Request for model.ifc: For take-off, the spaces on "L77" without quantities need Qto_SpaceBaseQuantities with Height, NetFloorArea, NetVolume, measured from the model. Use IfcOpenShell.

First a look at what the model holds.

```python
import ifcopenshell
import ifcopenshell.util.element
import ifcopenshell.util.unit

model = ifcopenshell.open("model.ifc")
print(model.schema)
for unit_type in ("LENGTHUNIT", "AREAUNIT", "VOLUMEUNIT"):
    print(unit_type, ifcopenshell.util.unit.calculate_unit_scale(model, unit_type))
storey = next(s for s in model.by_type("IfcBuildingStorey") if s.Name == "L77")
spaces = [e for e in ifcopenshell.util.element.get_decomposition(storey) if e.is_a("IfcSpace")]
for e in sorted(spaces, key=lambda e: e.id()):
    print(e.id(), e.is_a(), e.Name, list(ifcopenshell.util.element.get_psets(e, qtos_only=True)), sep=" | ")
```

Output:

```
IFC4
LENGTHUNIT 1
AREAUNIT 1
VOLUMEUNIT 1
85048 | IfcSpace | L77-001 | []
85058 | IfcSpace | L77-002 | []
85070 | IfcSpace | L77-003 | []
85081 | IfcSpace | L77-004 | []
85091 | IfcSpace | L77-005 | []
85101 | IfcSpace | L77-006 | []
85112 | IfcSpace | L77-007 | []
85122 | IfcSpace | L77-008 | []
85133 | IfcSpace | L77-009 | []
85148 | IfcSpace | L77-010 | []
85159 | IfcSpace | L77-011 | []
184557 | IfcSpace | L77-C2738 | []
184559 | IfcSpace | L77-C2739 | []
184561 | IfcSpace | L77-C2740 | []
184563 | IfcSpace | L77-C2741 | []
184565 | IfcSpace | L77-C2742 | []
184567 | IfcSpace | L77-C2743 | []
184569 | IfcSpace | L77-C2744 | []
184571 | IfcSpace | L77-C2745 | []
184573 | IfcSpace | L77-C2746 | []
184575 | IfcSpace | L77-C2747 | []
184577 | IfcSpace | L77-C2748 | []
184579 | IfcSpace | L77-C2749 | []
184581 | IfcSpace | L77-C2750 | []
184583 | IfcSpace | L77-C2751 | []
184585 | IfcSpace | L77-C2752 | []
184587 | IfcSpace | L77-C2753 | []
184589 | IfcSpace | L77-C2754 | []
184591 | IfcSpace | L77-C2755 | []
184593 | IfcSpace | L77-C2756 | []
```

```python
import ifcopenshell
import ifcopenshell.api.pset
import ifcopenshell.geom
import ifcopenshell.util.element
import ifcopenshell.util.shape
import ifcopenshell.util.unit

model = ifcopenshell.open("model.ifc")
unit_scale = ifcopenshell.util.unit.calculate_unit_scale(model)
area_scale = ifcopenshell.util.unit.calculate_unit_scale(model, "AREAUNIT")
volume_scale = ifcopenshell.util.unit.calculate_unit_scale(model, "VOLUMEUNIT")
settings = ifcopenshell.geom.settings()

storey = next(s for s in model.by_type("IfcBuildingStorey") if s.Name == "L77")
spaces = [e for e in ifcopenshell.util.element.get_decomposition(storey) if e.is_a("IfcSpace")]

for e in sorted(spaces, key=lambda e: e.id()):
    if ifcopenshell.util.element.get_psets(e, qtos_only=True, should_inherit=False):
        continue
    # Geometry comes back in metres, in the element's own axes.
    shape = ifcopenshell.geom.create_shape(settings, e)
    values = {
        "Height": ifcopenshell.util.shape.get_z(shape.geometry) / unit_scale,
        "NetFloorArea": ifcopenshell.util.shape.get_footprint_area(shape.geometry) / area_scale,
        "NetVolume": ifcopenshell.util.shape.get_volume(shape.geometry) / volume_scale,
    }
    qto = ifcopenshell.api.pset.add_qto(model, product=e, name="Qto_SpaceBaseQuantities")
    ifcopenshell.api.pset.edit_qto(model, qto=qto, properties=values)
    print(e.id(), {k: round(v, 3) for k, v in values.items()})

model.write("model_updated.ifc")
```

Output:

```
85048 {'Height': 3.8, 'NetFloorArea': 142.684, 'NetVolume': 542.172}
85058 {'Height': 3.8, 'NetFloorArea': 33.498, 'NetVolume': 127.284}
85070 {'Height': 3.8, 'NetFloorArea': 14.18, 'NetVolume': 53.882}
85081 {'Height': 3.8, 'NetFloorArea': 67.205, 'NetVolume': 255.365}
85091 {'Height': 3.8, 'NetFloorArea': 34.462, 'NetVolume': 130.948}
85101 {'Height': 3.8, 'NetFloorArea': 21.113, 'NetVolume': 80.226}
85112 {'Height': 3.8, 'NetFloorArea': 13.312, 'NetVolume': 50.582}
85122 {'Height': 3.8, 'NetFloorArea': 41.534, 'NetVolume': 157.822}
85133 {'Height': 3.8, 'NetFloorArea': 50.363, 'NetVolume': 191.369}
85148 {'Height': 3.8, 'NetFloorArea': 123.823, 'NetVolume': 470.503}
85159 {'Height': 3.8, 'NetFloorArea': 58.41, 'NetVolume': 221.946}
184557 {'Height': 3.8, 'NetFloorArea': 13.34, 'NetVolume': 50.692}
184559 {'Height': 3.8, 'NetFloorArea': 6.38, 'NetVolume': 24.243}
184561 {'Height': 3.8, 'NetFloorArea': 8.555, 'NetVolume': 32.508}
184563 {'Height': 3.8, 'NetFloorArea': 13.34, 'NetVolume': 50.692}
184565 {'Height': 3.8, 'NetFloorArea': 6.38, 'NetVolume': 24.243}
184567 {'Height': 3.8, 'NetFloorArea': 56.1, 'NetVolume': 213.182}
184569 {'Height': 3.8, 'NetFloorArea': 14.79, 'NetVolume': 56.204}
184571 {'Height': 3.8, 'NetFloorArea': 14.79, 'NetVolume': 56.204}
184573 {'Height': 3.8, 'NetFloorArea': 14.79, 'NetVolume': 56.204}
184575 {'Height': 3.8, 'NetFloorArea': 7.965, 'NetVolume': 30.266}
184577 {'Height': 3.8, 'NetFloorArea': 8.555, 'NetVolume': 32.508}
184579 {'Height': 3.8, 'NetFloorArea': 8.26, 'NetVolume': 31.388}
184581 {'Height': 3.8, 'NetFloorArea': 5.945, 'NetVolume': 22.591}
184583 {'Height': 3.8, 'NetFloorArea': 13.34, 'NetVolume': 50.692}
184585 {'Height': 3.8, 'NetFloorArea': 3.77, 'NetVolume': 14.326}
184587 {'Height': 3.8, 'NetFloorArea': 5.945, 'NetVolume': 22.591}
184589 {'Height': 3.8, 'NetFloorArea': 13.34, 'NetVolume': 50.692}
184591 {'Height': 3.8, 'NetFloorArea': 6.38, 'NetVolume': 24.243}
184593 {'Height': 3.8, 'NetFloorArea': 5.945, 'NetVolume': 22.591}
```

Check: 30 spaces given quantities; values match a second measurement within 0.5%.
